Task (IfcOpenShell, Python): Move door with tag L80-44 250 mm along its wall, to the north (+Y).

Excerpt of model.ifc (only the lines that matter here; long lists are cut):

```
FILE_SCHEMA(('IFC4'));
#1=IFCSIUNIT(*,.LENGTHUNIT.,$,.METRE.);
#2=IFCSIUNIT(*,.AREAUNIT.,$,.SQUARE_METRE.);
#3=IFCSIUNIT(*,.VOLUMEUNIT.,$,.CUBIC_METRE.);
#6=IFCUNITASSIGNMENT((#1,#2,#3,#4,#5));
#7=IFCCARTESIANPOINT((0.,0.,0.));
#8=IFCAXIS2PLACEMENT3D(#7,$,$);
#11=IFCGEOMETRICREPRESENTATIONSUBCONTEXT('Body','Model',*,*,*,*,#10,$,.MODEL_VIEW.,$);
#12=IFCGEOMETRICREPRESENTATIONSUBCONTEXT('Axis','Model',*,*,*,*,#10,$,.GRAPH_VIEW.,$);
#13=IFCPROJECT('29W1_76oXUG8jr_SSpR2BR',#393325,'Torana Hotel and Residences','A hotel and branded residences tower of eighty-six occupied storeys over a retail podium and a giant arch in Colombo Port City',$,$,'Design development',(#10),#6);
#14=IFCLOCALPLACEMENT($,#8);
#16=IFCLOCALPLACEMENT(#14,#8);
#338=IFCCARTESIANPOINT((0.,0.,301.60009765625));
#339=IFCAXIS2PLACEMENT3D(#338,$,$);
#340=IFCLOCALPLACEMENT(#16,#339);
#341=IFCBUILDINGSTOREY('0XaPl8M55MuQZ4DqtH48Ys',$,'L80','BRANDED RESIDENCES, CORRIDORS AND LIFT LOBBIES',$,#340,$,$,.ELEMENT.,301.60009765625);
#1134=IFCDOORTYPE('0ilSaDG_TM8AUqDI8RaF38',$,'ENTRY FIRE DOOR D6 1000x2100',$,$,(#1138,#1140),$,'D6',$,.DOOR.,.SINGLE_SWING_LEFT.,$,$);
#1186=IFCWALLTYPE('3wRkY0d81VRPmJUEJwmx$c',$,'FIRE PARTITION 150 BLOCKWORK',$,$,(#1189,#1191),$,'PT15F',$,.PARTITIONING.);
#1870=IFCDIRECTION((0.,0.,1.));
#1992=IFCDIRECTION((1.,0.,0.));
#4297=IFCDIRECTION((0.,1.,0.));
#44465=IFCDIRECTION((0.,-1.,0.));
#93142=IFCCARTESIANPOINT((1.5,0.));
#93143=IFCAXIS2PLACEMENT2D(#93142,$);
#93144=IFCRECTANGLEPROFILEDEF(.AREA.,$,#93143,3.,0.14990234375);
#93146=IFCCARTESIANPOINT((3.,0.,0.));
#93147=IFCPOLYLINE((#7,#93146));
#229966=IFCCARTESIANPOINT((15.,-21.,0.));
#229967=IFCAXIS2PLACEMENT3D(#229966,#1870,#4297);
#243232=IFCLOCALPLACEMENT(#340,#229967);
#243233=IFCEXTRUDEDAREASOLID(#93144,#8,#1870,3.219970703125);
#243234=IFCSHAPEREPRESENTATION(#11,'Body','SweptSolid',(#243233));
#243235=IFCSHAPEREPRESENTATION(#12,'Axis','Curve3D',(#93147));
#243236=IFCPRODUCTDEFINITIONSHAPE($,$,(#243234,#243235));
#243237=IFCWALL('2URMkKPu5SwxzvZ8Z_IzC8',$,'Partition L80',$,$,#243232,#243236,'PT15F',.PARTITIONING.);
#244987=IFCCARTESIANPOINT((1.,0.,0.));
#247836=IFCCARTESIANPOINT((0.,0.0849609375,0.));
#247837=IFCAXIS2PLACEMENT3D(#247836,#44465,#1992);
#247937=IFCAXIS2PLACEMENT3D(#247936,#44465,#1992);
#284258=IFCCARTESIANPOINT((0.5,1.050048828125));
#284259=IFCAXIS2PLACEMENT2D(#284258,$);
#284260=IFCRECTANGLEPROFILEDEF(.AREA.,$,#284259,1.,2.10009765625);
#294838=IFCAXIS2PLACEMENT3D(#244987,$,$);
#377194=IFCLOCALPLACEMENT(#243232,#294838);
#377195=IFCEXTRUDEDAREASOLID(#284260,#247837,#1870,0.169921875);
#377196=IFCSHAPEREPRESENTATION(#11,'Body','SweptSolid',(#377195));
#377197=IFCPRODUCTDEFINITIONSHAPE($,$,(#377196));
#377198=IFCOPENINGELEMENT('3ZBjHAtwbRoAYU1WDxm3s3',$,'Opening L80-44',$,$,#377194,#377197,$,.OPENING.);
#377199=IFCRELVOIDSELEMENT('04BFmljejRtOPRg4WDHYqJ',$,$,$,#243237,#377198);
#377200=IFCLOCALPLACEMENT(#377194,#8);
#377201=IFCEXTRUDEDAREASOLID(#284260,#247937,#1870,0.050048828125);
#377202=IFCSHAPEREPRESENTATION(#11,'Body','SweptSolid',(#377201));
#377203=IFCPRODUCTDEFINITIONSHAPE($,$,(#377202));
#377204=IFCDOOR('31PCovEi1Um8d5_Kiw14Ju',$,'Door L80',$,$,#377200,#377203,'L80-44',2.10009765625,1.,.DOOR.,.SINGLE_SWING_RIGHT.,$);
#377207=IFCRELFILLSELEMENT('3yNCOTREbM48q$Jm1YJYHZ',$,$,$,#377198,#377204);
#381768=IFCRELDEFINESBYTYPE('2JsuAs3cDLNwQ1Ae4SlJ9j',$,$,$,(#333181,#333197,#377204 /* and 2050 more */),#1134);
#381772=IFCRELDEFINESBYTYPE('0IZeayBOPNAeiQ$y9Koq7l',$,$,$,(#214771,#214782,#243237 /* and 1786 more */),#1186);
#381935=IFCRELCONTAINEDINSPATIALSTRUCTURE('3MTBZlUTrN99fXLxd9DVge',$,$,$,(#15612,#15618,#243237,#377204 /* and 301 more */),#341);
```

```python
import ifcopenshell
import ifcopenshell.api.geometry
import ifcopenshell.util.placement
import ifcopenshell.util.unit

model = ifcopenshell.open("model.ifc")
unit_scale = ifcopenshell.util.unit.calculate_unit_scale(model)

door = model.by_guid("31PCovEi1Um8d5_Kiw14Ju")
opening = door.FillsVoids[0].RelatingOpeningElement
wall = opening.VoidsElements[0].RelatingBuildingElement

wall_matrix = ifcopenshell.util.placement.get_local_placement(wall.ObjectPlacement)
shift = wall_matrix[:3, 0] * 0.25 / unit_scale
before = ifcopenshell.util.placement.get_local_placement(door.ObjectPlacement)[:3, 3].copy()

# The door is placed relative to its opening, so it follows when the opening moves.
matrix = ifcopenshell.util.placement.get_local_placement(opening.ObjectPlacement)
matrix[:3, 3] += shift
ifcopenshell.api.geometry.edit_object_placement(
    model, product=opening, matrix=matrix, is_si=False, should_transform_children=True
)

after = ifcopenshell.util.placement.get_local_placement(door.ObjectPlacement)[:3, 3]
print("door moved by", (after - before).round(3) + 0.0)

model.write("model_v2.ifc")
```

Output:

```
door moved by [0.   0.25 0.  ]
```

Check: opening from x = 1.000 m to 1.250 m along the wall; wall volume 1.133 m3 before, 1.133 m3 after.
